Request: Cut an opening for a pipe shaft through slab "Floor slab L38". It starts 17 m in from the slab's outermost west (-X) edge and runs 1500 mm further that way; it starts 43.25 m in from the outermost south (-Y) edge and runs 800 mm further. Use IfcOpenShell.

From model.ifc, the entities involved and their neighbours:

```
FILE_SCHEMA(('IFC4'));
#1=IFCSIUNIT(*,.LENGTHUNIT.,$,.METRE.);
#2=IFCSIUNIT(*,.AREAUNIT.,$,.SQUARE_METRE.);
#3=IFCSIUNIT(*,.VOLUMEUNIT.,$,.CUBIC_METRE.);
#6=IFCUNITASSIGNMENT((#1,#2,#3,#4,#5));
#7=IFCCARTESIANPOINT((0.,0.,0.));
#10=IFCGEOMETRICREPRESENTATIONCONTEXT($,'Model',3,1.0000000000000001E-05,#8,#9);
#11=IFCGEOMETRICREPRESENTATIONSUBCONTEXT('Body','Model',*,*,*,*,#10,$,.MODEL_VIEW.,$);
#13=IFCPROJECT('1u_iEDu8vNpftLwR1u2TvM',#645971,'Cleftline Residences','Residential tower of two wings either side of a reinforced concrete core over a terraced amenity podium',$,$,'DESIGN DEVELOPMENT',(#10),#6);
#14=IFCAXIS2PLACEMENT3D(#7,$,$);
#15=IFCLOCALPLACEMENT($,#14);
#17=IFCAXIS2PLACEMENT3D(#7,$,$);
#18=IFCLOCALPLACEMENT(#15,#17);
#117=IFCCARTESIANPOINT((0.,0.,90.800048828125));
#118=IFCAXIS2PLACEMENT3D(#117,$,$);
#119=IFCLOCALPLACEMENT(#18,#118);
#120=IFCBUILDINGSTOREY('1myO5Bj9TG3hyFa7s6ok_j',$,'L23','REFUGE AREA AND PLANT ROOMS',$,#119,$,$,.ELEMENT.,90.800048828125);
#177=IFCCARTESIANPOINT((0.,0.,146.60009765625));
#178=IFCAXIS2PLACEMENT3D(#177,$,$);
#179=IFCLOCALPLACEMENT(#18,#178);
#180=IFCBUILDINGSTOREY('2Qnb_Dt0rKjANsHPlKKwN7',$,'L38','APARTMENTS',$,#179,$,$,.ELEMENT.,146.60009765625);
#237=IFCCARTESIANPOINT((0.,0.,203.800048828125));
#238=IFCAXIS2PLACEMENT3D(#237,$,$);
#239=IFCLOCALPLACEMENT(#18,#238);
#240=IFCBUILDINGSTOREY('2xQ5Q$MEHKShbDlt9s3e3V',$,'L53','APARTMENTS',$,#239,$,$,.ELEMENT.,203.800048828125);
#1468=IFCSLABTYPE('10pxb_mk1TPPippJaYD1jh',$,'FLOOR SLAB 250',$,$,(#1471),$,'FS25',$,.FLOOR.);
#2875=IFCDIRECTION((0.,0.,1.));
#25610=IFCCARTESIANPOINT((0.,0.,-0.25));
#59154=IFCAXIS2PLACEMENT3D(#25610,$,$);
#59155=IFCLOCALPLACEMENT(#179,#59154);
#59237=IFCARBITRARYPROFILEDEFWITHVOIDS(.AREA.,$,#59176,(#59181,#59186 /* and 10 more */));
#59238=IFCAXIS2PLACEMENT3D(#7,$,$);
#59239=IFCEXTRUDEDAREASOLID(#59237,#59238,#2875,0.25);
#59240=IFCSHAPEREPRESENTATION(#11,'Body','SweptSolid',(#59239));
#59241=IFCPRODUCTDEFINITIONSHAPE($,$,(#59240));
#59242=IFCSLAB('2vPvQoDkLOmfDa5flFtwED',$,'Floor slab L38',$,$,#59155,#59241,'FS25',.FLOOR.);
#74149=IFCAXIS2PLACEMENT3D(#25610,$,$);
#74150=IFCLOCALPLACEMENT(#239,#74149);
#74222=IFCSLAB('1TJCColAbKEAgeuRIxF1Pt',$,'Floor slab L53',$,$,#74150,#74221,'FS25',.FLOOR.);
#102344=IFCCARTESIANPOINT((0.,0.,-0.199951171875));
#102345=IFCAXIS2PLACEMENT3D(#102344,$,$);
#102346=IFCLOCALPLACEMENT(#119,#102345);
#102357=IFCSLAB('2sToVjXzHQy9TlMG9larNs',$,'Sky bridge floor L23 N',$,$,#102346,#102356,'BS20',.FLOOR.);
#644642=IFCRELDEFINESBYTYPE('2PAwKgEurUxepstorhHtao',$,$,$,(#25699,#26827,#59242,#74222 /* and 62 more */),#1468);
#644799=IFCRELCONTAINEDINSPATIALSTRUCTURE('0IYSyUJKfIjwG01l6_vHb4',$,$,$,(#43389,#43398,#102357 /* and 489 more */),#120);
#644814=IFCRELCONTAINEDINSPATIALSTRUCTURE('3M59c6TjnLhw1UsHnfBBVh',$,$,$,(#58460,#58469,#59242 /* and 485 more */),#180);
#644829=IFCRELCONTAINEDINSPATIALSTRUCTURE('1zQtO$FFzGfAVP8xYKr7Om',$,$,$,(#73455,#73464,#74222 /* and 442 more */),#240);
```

```python
import numpy as np
import ifcopenshell
import ifcopenshell.api.feature
import ifcopenshell.api.geometry
import ifcopenshell.api.root
import ifcopenshell.geom
import ifcopenshell.util.placement
import ifcopenshell.util.representation
import ifcopenshell.util.shape
import ifcopenshell.util.unit

model = ifcopenshell.open("model.ifc")
unit_scale = ifcopenshell.util.unit.calculate_unit_scale(model)
settings = ifcopenshell.geom.settings()


def volume(element):
    """Net volume in cubic metres, openings subtracted."""
    shape = ifcopenshell.geom.create_shape(settings, element)
    return ifcopenshell.util.shape.get_volume(shape.geometry)


slab = model.by_guid("2vPvQoDkLOmfDa5flFtwED")
before = volume(slab)

# Extent in the slab's own axes, in metres. The edges named are its -X and -Y sides.
slab_shape = ifcopenshell.geom.create_shape(settings, slab)
vertices = ifcopenshell.util.shape.get_vertices(slab_shape.geometry)
x_min, y_min, bottom = vertices.min(axis=0)
top = vertices[:, 2].max()

opening = ifcopenshell.api.root.create_entity(model, ifc_class="IfcOpeningElement", name="Pipe shaft opening", predefined_type="OPENING")
context = ifcopenshell.util.representation.get_context(model, "Model", "Body", "MODEL_VIEW")
width, depth = 1.5, 0.8
outline = [(0.0, 0.0), (width, 0.0), (width, depth), (0.0, depth), (0.0, 0.0)]
# Overshoot both faces by 50 mm so the cut is clean.
shape = ifcopenshell.api.geometry.add_slab_representation(
    model, context=context, depth=top - bottom + 0.1, polyline=outline
)
ifcopenshell.api.geometry.assign_representation(model, product=opening, representation=shape)

matrix = ifcopenshell.util.placement.get_local_placement(slab.ObjectPlacement)
matrix[:, 3] = matrix @ np.append(np.array([x_min + 17, y_min + 43.25, bottom - 0.05]) / unit_scale, 1.0)
ifcopenshell.api.geometry.edit_object_placement(model, product=opening, matrix=matrix, is_si=False)
ifcopenshell.api.feature.add_feature(model, feature=opening, element=slab)

after = volume(slab)

print(f"slab volume {before:.3f} -> {after:.3f} m3")

model.write("model_rev.ifc")
```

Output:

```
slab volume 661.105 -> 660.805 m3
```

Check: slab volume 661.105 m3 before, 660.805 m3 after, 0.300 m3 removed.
